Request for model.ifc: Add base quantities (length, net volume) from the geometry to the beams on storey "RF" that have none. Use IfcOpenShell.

First a look at what the model holds.

```python
import ifcopenshell
import ifcopenshell.util.element
import ifcopenshell.util.unit

model = ifcopenshell.open("model.ifc")
print(model.schema)
for unit_type in ("LENGTHUNIT", "AREAUNIT", "VOLUMEUNIT"):
    print(unit_type, ifcopenshell.util.unit.calculate_unit_scale(model, unit_type))
storey = next(s for s in model.by_type("IfcBuildingStorey") if s.Name == "RF")
beams = [e for e in ifcopenshell.util.element.get_decomposition(storey) if e.is_a("IfcBeam")]
for e in sorted(beams, key=lambda e: e.id()):
    print(e.id(), e.is_a(), e.Name, list(ifcopenshell.util.element.get_psets(e, qtos_only=True)), sep=" | ")
```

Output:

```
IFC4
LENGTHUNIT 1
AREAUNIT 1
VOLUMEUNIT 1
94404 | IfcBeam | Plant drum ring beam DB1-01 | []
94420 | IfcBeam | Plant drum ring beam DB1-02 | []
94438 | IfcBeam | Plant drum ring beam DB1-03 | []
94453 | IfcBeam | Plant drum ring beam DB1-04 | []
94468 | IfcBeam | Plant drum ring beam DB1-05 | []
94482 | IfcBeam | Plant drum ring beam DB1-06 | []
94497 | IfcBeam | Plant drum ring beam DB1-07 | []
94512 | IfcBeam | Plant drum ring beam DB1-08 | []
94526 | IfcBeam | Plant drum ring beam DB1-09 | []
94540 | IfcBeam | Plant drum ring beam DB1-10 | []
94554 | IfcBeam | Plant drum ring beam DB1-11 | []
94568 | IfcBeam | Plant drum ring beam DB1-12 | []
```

```python
import ifcopenshell
import ifcopenshell.api.pset
import ifcopenshell.geom
import ifcopenshell.util.element
import ifcopenshell.util.shape
import ifcopenshell.util.unit

model = ifcopenshell.open("model.ifc")
unit_scale = ifcopenshell.util.unit.calculate_unit_scale(model)
volume_scale = ifcopenshell.util.unit.calculate_unit_scale(model, "VOLUMEUNIT")
settings = ifcopenshell.geom.settings()

storey = next(s for s in model.by_type("IfcBuildingStorey") if s.Name == "RF")
beams = [e for e in ifcopenshell.util.element.get_decomposition(storey) if e.is_a("IfcBeam")]

for e in sorted(beams, key=lambda e: e.id()):
    if ifcopenshell.util.element.get_psets(e, qtos_only=True, should_inherit=False):
        continue
    # Geometry comes back in metres, in the element's own axes.
    shape = ifcopenshell.geom.create_shape(settings, e)
    values = {
        "Length": ifcopenshell.util.shape.get_max_xyz(shape.geometry) / unit_scale,
        "NetVolume": ifcopenshell.util.shape.get_volume(shape.geometry) / volume_scale,
    }
    qto = ifcopenshell.api.pset.add_qto(model, product=e, name="Qto_BeamBaseQuantities")
    ifcopenshell.api.pset.edit_qto(model, qto=qto, properties=values)
    print(e.id(), {k: round(v, 3) for k, v in values.items()})

model.write("model-out.ifc")
```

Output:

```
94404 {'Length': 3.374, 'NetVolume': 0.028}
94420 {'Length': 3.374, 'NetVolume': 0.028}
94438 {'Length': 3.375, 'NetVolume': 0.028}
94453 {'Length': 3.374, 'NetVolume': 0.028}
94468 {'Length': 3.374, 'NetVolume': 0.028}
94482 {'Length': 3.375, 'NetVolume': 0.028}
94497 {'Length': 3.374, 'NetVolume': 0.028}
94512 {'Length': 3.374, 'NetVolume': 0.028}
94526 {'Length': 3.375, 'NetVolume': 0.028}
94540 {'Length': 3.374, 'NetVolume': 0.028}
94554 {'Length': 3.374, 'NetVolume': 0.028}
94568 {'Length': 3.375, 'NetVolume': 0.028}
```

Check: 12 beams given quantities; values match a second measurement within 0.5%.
